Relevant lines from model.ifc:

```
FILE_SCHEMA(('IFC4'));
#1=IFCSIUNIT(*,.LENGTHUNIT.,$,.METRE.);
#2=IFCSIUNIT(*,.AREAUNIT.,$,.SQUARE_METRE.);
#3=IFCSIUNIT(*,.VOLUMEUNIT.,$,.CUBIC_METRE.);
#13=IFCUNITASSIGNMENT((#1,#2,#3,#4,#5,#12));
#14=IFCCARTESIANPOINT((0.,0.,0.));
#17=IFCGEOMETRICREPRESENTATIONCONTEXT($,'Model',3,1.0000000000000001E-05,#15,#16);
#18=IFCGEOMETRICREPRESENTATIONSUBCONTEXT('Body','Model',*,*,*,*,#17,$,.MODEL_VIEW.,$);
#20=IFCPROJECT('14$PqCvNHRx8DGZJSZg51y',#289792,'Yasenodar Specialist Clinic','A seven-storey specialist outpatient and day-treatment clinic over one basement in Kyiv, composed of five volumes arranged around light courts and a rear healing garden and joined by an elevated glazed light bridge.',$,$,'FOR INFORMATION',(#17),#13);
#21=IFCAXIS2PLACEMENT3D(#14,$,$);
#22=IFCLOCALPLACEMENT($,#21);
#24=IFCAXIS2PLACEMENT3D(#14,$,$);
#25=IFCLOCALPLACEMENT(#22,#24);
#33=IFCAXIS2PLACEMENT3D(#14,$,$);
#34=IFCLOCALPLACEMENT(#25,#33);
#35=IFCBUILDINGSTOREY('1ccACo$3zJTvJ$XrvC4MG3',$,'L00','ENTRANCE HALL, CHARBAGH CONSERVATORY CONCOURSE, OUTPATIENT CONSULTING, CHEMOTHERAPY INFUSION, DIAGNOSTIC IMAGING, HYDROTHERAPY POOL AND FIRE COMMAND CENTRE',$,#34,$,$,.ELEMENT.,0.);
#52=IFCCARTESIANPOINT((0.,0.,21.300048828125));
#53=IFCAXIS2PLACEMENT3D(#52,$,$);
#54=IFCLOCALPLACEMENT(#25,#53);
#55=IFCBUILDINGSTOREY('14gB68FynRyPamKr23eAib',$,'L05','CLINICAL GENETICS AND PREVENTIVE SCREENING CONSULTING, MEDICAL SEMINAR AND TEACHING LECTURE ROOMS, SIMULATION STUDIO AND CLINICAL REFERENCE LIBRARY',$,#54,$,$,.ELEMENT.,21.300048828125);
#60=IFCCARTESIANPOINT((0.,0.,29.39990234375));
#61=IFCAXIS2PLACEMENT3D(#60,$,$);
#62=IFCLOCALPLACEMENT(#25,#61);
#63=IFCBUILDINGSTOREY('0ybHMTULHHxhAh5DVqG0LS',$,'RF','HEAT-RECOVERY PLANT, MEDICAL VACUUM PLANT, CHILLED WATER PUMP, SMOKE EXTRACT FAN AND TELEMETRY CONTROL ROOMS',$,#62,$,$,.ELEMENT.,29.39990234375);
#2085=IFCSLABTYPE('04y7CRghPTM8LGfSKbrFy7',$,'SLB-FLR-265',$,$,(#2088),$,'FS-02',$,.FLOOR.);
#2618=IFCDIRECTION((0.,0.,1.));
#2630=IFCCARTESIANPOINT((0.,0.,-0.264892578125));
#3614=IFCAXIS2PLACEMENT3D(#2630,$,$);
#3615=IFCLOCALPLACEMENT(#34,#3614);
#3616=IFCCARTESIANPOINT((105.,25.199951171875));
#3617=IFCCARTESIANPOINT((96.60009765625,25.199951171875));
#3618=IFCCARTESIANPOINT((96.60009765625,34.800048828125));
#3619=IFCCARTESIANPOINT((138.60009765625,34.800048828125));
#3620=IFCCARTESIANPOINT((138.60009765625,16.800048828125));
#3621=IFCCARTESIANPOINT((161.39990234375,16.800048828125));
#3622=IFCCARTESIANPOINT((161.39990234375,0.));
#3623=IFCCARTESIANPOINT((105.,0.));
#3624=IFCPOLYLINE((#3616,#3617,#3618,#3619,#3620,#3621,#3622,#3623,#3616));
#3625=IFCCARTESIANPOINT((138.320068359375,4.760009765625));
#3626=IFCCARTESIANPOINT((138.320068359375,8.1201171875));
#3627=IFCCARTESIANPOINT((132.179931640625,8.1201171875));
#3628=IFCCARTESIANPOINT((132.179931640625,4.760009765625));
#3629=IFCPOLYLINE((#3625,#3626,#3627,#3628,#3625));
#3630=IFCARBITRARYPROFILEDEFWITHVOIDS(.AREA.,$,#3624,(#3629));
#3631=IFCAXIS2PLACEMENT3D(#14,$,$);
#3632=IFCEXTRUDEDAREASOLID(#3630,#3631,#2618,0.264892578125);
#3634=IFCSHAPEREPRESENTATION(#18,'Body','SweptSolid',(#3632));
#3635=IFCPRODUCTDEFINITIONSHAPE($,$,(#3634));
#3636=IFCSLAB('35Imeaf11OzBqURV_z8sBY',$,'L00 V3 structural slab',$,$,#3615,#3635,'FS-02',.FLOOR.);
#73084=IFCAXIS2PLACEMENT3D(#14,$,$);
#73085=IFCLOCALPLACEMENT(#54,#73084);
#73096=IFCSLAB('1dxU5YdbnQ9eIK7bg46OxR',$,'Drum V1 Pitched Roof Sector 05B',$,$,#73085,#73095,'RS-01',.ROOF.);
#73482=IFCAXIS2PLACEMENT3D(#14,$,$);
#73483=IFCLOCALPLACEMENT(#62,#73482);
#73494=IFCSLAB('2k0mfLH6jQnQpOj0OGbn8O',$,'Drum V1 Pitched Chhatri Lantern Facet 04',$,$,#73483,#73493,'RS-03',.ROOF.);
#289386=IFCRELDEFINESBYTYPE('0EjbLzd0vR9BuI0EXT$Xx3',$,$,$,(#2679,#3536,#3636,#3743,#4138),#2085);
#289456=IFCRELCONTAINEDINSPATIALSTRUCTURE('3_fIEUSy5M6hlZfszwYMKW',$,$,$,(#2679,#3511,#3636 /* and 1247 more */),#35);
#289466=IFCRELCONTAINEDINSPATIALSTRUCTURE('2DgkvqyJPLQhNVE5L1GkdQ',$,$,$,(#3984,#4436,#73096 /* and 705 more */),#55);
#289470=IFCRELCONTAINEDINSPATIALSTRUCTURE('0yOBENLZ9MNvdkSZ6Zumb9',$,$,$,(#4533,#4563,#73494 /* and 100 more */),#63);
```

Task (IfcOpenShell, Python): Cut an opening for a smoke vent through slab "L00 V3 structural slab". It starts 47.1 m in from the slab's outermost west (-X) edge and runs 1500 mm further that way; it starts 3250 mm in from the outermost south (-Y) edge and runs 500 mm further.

```python
import numpy as np
import ifcopenshell
import ifcopenshell.api.feature
import ifcopenshell.api.geometry
import ifcopenshell.api.root
import ifcopenshell.geom
import ifcopenshell.util.placement
import ifcopenshell.util.representation
import ifcopenshell.util.shape
import ifcopenshell.util.unit

model = ifcopenshell.open("model.ifc")
unit_scale = ifcopenshell.util.unit.calculate_unit_scale(model)
settings = ifcopenshell.geom.settings()


def volume(element):
    """Net volume in cubic metres, openings subtracted."""
    shape = ifcopenshell.geom.create_shape(settings, element)
    return ifcopenshell.util.shape.get_volume(shape.geometry)


slab = model.by_id(3636)
before = volume(slab)

# Extent in the slab's own axes, in metres. The edges named are its -X and -Y sides.
slab_shape = ifcopenshell.geom.create_shape(settings, slab)
vertices = ifcopenshell.util.shape.get_vertices(slab_shape.geometry)
x_min, y_min, bottom = vertices.min(axis=0)
top = vertices[:, 2].max()

opening = ifcopenshell.api.root.create_entity(model, ifc_class="IfcOpeningElement", name="Smoke vent opening", predefined_type="OPENING")
context = ifcopenshell.util.representation.get_context(model, "Model", "Body", "MODEL_VIEW")
width, depth = 1.5, 0.5
outline = [(0.0, 0.0), (width, 0.0), (width, depth), (0.0, depth), (0.0, 0.0)]
# Overshoot both faces by 50 mm so the cut is clean.
shape = ifcopenshell.api.geometry.add_slab_representation(
    model, context=context, depth=top - bottom + 0.1, polyline=outline
)
ifcopenshell.api.geometry.assign_representation(model, product=opening, representation=shape)

matrix = ifcopenshell.util.placement.get_local_placement(slab.ObjectPlacement)
matrix[:, 3] = matrix @ np.append(np.array([x_min + 47.1, y_min + 3.25, bottom - 0.05]) / unit_scale, 1.0)
ifcopenshell.api.geometry.edit_object_placement(model, product=opening, matrix=matrix, is_si=False)
ifcopenshell.api.feature.add_feature(model, feature=opening, element=slab)

after = volume(slab)

print(f"slab volume {before:.3f} -> {after:.3f} m3")

model.write("model_v2.ifc")
```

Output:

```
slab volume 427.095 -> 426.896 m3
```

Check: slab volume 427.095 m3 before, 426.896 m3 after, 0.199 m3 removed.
